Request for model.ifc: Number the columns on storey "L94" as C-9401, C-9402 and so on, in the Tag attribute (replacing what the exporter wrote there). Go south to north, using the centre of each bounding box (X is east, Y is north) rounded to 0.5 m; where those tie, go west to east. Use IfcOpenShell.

First a look at what the model holds.

```python
import ifcopenshell
import ifcopenshell.util.element
import ifcopenshell.util.placement

model = ifcopenshell.open("model.ifc")
print(model.schema)
storey = next(s for s in model.by_type("IfcBuildingStorey") if s.Name == "L94")
columns = [e for e in ifcopenshell.util.element.get_decomposition(storey) if e.is_a("IfcColumn")]
for e in sorted(columns, key=lambda e: e.id()):
    origin = ifcopenshell.util.placement.get_local_placement(e.ObjectPlacement)[:3, 3]
    print(e.id(), e.Tag, e.Name, origin.round(2) + 0.0, sep=" | ")
```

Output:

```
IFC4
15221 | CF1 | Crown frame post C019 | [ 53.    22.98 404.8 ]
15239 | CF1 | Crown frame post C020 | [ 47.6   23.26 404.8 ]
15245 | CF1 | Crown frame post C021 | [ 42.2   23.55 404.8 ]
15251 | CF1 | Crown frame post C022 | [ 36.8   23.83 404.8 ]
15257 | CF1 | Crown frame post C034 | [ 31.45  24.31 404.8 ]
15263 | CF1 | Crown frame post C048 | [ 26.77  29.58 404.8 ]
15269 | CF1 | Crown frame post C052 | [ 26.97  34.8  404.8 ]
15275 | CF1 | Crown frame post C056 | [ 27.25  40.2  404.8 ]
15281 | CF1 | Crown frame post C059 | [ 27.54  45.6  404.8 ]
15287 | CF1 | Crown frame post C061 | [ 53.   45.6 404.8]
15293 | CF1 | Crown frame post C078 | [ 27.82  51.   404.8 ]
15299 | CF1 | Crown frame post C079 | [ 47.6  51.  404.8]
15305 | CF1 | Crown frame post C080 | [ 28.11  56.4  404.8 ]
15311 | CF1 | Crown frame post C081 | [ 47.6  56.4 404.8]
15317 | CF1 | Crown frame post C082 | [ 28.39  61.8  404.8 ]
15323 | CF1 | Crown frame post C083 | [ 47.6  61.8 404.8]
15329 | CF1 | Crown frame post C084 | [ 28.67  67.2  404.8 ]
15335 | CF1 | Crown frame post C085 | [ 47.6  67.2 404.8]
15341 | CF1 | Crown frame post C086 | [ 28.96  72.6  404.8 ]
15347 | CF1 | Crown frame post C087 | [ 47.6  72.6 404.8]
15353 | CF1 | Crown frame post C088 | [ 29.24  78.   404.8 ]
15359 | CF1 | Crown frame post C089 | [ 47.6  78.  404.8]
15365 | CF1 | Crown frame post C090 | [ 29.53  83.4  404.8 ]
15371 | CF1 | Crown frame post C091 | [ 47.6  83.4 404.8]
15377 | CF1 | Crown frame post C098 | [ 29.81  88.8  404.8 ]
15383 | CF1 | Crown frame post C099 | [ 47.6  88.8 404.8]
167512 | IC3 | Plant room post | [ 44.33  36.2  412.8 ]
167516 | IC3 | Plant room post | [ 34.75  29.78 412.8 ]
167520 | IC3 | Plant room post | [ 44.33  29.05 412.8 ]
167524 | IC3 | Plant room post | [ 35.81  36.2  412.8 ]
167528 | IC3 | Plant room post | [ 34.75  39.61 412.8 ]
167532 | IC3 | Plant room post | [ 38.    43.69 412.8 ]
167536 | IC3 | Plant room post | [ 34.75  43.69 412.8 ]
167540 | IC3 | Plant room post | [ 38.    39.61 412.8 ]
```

```python
import ifcopenshell
import ifcopenshell.geom
import ifcopenshell.util.element
import ifcopenshell.util.shape

model = ifcopenshell.open("model.ifc")
settings = ifcopenshell.geom.settings()
settings.set("use-world-coords", True)


def centre(element):
    shape = ifcopenshell.geom.create_shape(settings, element)
    return ifcopenshell.util.shape.get_bbox_centroid(shape.geometry)


storey = next(s for s in model.by_type("IfcBuildingStorey") if s.Name == "L94")
columns = [e for e in ifcopenshell.util.element.get_decomposition(storey) if e.is_a("IfcColumn")]

# Insertion points can sit at a corner or the storey origin, so sort by the geometry (in metres).
centres = {e: centre(e) for e in columns}
columns.sort(key=lambda e: (round(centres[e][1] / 0.5), centres[e][0]))

for i, e in enumerate(columns, start=1):
    number = f"C-94{i:02d}"
    e.Tag = number
    print(e.id(), number)

model.write("model-out.ifc")
```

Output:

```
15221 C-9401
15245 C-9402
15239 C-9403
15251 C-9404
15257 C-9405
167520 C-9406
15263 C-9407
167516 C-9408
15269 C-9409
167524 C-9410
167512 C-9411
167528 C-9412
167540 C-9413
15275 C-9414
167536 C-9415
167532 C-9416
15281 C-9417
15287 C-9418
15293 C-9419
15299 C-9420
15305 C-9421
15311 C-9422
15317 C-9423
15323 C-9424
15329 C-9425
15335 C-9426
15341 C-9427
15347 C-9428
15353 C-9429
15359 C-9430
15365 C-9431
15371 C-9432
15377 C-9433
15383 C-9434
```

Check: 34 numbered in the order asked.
